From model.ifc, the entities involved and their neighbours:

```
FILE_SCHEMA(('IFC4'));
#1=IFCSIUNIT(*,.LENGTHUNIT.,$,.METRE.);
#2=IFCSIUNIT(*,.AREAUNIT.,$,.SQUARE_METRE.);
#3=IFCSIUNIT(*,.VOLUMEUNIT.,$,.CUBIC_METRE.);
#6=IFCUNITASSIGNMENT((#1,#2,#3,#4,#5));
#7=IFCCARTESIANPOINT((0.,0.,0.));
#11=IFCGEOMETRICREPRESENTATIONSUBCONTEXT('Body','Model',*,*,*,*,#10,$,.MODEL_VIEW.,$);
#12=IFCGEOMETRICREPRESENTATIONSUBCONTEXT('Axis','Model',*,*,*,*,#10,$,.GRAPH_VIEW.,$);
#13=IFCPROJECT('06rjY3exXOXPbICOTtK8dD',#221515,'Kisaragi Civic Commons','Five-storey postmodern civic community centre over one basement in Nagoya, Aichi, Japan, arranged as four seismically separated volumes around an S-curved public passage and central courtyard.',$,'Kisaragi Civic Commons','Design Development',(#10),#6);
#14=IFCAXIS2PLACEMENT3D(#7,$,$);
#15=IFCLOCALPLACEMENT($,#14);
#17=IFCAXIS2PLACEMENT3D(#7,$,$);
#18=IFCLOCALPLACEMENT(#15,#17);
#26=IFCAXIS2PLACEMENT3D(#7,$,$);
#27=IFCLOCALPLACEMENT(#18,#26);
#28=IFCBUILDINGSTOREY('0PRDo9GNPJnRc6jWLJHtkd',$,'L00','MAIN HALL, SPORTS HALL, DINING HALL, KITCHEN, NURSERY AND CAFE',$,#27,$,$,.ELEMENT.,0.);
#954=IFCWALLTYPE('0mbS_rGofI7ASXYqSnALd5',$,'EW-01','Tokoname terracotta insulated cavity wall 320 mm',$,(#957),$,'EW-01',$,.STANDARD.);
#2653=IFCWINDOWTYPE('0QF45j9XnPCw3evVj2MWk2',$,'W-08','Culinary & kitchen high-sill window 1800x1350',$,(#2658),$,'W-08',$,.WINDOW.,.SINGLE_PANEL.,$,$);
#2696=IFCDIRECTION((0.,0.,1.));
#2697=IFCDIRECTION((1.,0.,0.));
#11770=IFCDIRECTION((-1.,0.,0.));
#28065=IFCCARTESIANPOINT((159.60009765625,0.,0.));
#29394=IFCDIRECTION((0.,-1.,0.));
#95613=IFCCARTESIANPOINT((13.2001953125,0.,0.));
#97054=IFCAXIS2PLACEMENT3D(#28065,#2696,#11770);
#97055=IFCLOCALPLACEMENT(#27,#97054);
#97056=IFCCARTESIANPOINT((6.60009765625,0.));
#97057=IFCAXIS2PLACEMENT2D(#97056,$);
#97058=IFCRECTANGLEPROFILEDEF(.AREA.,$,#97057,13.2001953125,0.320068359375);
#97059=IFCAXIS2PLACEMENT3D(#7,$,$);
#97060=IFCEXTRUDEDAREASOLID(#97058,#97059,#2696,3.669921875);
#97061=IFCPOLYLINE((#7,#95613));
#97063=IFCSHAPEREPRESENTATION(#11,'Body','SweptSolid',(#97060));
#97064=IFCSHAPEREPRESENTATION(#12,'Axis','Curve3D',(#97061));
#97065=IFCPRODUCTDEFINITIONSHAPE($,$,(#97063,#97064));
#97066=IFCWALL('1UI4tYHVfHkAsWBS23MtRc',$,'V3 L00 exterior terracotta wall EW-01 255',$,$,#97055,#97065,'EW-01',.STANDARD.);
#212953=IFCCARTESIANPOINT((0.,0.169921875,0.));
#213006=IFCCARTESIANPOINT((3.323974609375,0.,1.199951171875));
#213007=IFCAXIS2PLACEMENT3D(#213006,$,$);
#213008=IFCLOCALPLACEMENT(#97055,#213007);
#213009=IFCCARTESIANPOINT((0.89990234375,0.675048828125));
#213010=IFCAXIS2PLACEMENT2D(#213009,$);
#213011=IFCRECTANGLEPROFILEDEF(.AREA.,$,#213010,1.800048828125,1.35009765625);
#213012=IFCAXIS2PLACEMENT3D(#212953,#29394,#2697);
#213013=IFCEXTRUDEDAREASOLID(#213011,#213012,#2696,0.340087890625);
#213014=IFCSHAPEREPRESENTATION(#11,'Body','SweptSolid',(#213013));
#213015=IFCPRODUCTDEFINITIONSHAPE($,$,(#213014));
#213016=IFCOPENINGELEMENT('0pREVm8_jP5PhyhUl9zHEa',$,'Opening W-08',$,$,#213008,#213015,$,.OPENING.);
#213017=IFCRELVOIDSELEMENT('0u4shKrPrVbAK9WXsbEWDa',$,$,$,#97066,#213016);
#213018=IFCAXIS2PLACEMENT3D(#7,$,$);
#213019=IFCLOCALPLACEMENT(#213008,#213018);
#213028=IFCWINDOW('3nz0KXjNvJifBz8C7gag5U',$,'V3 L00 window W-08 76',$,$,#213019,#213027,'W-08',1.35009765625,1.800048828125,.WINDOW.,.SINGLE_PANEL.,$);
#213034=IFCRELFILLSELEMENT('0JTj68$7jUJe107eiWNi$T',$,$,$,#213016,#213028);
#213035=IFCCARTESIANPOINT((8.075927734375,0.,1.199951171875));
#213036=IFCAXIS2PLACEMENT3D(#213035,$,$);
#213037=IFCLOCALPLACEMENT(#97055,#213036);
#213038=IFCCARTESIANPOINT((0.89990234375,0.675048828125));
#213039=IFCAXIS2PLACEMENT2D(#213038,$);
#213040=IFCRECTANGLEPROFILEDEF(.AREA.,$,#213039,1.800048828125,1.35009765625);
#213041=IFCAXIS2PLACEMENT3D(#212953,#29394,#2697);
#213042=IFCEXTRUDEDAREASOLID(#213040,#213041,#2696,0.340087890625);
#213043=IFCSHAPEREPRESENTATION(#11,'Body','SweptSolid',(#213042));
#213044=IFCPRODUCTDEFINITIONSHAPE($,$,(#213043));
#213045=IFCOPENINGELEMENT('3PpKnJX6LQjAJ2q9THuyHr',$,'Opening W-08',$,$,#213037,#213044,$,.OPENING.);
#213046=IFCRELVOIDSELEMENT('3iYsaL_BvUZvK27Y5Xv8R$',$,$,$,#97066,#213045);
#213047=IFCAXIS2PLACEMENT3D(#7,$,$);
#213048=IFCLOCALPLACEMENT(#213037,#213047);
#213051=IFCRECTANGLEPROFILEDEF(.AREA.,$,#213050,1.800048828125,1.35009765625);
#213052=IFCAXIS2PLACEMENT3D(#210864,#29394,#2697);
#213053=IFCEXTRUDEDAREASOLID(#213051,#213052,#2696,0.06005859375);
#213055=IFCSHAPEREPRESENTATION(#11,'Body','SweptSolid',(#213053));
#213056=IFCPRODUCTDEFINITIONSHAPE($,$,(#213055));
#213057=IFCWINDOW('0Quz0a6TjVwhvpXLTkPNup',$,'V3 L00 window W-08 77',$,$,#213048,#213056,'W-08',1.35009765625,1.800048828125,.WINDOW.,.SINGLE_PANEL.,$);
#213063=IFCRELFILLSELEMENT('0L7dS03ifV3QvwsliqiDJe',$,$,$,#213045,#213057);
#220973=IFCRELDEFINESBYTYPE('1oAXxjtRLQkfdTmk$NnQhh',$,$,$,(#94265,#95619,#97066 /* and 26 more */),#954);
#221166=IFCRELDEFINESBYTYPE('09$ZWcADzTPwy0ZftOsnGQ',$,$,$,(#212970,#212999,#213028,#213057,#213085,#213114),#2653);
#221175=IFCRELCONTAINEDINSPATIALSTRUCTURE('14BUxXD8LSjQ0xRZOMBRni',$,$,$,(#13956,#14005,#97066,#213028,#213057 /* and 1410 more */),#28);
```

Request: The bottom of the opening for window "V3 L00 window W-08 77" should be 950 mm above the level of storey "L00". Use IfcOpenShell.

```python
import numpy as np
import ifcopenshell
import ifcopenshell.api.geometry
import ifcopenshell.geom
import ifcopenshell.util.element
import ifcopenshell.util.placement
import ifcopenshell.util.shape
import ifcopenshell.util.unit

model = ifcopenshell.open("model.ifc")
unit_scale = ifcopenshell.util.unit.calculate_unit_scale(model)

window = model.by_id(213057)
opening = window.FillsVoids[0].RelatingOpeningElement
storey = ifcopenshell.util.element.get_container(window, ifc_class="IfcBuildingStorey")
level = ifcopenshell.util.placement.get_local_placement(storey.ObjectPlacement)[2, 3]

# The opening's origin need not be at the sill, so measure its lowest point.
shape = ifcopenshell.geom.create_shape(ifcopenshell.geom.settings(), opening)
bottom = ifcopenshell.util.shape.get_shape_bottom_elevation(shape, shape.geometry) / unit_scale
dz = level + 0.95 / unit_scale - bottom

shift = np.array([0.0, 0.0, dz])
# The window is placed relative to its opening, so it follows when the opening moves.
matrix = ifcopenshell.util.placement.get_local_placement(opening.ObjectPlacement)
matrix[:3, 3] += shift
ifcopenshell.api.geometry.edit_object_placement(
    model, product=opening, matrix=matrix, is_si=False, should_transform_children=True
)

print(f"moved by {dz * unit_scale:+.3f} m")

model.write("model_rev.ifc")
```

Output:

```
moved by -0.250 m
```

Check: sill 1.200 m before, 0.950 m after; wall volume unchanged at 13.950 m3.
